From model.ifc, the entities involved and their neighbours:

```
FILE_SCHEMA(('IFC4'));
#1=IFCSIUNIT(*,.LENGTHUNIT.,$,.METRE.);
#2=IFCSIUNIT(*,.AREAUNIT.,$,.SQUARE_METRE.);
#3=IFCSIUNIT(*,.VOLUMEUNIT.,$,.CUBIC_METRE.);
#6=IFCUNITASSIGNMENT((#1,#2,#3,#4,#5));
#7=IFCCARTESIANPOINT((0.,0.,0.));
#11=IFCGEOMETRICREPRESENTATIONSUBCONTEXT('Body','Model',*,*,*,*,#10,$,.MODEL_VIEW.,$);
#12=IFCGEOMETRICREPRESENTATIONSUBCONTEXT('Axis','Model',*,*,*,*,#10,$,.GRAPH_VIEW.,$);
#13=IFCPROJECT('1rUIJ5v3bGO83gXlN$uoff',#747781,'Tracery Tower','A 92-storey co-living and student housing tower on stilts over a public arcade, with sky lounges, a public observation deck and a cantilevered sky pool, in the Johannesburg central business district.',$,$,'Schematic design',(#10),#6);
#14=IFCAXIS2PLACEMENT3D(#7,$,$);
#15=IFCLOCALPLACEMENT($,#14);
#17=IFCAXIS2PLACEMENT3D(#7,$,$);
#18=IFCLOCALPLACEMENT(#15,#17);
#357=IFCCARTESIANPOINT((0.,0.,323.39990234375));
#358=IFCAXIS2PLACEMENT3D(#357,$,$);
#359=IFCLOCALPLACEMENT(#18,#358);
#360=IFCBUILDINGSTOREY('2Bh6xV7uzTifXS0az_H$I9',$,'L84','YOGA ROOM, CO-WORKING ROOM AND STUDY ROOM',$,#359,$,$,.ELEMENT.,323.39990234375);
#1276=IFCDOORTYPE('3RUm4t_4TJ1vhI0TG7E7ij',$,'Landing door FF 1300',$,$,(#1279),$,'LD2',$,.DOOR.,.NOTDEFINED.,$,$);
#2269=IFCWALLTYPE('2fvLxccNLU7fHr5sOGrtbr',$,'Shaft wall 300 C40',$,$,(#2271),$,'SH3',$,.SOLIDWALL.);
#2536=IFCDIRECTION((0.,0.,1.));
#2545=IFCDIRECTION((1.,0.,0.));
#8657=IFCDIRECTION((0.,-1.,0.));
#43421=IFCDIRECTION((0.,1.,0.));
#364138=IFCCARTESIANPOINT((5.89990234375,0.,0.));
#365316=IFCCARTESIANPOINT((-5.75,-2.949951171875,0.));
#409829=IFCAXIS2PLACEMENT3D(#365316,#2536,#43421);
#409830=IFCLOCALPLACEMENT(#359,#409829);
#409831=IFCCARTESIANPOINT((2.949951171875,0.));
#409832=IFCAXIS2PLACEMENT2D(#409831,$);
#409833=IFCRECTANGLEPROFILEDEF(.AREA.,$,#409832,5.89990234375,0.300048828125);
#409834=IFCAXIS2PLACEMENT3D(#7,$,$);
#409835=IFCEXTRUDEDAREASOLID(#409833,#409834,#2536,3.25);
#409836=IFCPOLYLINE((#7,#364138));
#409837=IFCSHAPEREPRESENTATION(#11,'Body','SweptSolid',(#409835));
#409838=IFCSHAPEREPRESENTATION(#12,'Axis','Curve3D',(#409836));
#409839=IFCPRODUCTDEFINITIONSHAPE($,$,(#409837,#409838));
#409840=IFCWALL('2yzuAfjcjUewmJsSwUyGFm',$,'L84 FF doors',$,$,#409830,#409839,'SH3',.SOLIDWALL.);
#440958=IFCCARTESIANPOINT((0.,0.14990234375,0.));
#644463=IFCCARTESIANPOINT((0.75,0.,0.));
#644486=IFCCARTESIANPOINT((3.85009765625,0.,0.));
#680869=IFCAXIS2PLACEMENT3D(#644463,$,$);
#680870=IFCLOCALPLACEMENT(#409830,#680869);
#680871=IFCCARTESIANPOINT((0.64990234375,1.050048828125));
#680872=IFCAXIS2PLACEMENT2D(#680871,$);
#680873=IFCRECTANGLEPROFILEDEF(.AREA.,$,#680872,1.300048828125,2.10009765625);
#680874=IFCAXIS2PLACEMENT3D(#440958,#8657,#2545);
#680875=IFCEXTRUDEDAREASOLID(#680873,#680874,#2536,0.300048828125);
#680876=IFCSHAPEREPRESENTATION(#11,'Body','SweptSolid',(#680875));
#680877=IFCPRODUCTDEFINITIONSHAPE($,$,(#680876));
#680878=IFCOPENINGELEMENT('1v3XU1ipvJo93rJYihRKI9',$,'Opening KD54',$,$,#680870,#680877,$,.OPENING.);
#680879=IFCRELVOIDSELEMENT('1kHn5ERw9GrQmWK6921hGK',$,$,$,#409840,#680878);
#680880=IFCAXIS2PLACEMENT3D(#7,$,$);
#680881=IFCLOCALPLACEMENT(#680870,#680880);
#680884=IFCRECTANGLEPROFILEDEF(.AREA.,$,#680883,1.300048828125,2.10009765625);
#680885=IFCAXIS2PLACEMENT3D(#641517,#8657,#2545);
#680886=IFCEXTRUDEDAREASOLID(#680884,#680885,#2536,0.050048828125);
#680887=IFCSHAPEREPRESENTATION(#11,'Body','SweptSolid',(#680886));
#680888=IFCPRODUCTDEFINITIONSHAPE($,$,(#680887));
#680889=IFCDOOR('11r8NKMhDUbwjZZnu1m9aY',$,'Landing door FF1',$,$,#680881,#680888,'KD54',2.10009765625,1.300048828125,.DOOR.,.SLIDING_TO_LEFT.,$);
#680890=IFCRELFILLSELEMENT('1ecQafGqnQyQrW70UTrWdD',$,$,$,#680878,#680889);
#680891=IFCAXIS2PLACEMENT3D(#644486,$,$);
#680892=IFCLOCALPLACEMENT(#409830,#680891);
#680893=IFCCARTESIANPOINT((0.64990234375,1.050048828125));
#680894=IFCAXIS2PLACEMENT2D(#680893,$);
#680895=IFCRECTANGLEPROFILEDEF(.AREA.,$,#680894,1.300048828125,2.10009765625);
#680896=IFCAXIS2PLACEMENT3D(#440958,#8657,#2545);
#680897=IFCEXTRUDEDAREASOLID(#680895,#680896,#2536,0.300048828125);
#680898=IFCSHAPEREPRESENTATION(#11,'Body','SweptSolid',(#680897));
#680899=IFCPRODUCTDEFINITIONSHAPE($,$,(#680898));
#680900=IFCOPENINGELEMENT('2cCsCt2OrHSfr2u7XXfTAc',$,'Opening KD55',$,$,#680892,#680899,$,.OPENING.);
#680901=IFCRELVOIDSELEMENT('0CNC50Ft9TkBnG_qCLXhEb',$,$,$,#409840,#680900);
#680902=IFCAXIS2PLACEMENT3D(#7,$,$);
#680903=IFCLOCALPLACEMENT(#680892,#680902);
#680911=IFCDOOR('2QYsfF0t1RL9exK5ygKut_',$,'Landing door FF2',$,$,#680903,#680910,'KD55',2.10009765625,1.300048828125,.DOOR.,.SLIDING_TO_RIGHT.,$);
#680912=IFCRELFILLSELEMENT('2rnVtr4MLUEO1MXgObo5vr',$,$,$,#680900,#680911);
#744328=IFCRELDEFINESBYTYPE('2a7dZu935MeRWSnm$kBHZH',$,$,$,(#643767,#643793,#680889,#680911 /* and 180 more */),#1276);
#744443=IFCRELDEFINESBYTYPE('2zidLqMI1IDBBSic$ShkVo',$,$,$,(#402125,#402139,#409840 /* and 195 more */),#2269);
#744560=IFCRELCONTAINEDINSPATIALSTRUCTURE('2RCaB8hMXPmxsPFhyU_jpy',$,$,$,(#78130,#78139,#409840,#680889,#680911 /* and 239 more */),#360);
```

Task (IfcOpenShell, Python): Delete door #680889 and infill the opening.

```python
import ifcopenshell
import ifcopenshell.api.feature
import ifcopenshell.api.root
import ifcopenshell.geom
import ifcopenshell.util.shape

model = ifcopenshell.open("model.ifc")
settings = ifcopenshell.geom.settings()


def volume(element):
    """Net volume in cubic metres, openings subtracted."""
    shape = ifcopenshell.geom.create_shape(settings, element)
    return ifcopenshell.util.shape.get_volume(shape.geometry)


door = model.by_guid("11r8NKMhDUbwjZZnu1m9aY")
opening = door.FillsVoids[0].RelatingOpeningElement
wall = opening.VoidsElements[0].RelatingBuildingElement
before = volume(wall)

ifcopenshell.api.root.remove_product(model, product=door)
ifcopenshell.api.feature.remove_feature(model, feature=opening)

after = volume(wall)

print(f"wall volume {before:.3f} -> {after:.3f} m3")

model.write("model_edited.ifc")
```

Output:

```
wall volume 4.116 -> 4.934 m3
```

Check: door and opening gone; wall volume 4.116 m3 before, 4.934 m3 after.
